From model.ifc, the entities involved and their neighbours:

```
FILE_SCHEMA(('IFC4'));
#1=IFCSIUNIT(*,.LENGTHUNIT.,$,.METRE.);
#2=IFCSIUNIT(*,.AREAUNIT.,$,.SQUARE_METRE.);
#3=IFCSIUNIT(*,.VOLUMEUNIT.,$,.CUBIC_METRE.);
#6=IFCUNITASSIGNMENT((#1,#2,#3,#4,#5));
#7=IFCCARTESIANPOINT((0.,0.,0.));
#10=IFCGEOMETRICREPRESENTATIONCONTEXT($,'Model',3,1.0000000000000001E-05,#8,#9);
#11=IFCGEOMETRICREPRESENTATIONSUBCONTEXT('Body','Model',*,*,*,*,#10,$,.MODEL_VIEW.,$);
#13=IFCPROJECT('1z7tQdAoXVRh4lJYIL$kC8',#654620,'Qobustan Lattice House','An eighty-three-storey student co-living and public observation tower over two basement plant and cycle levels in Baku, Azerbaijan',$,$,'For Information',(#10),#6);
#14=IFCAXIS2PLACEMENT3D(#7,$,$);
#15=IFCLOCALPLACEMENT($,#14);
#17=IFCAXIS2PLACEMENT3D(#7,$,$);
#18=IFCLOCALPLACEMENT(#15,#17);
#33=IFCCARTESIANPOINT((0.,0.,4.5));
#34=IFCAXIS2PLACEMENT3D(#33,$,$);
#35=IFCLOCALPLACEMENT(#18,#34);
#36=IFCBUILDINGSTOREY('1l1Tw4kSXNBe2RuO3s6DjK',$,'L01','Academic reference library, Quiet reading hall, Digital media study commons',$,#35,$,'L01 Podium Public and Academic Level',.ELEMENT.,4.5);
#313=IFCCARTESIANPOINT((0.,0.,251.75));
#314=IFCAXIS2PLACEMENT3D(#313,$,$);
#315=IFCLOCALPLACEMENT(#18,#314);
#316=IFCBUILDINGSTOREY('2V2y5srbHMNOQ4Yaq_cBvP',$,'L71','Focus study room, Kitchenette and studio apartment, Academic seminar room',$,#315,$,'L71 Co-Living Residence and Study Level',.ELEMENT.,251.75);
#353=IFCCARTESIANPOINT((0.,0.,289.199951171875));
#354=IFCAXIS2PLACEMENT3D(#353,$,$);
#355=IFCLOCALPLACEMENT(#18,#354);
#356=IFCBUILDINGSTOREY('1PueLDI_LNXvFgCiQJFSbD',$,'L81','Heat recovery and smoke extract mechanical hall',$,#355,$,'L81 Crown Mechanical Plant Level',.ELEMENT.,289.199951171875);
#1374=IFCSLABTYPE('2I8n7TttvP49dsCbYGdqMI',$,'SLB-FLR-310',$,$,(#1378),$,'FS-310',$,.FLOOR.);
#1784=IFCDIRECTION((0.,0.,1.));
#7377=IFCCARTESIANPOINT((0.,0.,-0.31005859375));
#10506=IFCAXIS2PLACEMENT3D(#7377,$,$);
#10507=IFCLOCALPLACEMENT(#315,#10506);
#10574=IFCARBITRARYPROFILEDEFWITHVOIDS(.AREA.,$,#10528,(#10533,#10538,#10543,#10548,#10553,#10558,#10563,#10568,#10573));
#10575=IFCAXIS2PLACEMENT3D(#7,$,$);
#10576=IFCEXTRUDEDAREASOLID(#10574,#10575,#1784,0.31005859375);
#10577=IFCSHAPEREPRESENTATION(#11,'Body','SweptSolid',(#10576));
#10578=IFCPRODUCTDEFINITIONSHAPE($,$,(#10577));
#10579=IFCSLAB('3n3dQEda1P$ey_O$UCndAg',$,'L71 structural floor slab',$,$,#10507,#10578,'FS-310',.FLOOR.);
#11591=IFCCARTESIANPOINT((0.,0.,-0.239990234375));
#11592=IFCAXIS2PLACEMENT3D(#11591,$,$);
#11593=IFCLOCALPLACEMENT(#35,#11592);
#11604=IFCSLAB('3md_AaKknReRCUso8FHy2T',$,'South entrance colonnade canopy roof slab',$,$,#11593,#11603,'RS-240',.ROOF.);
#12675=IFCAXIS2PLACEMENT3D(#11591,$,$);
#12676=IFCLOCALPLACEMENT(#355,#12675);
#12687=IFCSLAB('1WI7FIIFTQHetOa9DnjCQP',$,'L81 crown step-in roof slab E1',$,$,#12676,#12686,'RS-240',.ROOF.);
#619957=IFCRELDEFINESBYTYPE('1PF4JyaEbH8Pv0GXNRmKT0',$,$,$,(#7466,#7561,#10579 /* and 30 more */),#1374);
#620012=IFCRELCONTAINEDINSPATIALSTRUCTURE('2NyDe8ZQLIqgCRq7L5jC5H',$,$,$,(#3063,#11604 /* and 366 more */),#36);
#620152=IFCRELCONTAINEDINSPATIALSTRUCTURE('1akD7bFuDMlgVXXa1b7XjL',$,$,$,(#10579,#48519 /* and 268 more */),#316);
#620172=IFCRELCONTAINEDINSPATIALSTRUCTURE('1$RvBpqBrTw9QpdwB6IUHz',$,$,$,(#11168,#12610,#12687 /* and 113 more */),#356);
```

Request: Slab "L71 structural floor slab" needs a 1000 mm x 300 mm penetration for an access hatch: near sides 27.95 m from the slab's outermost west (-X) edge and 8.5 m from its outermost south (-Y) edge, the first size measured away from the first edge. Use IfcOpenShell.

```python
import numpy as np
import ifcopenshell
import ifcopenshell.api.feature
import ifcopenshell.api.geometry
import ifcopenshell.api.root
import ifcopenshell.geom
import ifcopenshell.util.placement
import ifcopenshell.util.representation
import ifcopenshell.util.shape
import ifcopenshell.util.unit

model = ifcopenshell.open("model.ifc")
unit_scale = ifcopenshell.util.unit.calculate_unit_scale(model)
settings = ifcopenshell.geom.settings()


def volume(element):
    """Net volume in cubic metres, openings subtracted."""
    shape = ifcopenshell.geom.create_shape(settings, element)
    return ifcopenshell.util.shape.get_volume(shape.geometry)


slab = model.by_guid("3n3dQEda1P$ey_O$UCndAg")
before = volume(slab)

# Extent in the slab's own axes, in metres. The edges named are its -X and -Y sides.
slab_shape = ifcopenshell.geom.create_shape(settings, slab)
vertices = ifcopenshell.util.shape.get_vertices(slab_shape.geometry)
x_min, y_min, bottom = vertices.min(axis=0)
top = vertices[:, 2].max()

opening = ifcopenshell.api.root.create_entity(model, ifc_class="IfcOpeningElement", name="Access hatch opening", predefined_type="OPENING")
context = ifcopenshell.util.representation.get_context(model, "Model", "Body", "MODEL_VIEW")
width, depth = 1, 0.3
outline = [(0.0, 0.0), (width, 0.0), (width, depth), (0.0, depth), (0.0, 0.0)]
# Overshoot both faces by 50 mm so the cut is clean.
shape = ifcopenshell.api.geometry.add_slab_representation(
    model, context=context, depth=top - bottom + 0.1, polyline=outline
)
ifcopenshell.api.geometry.assign_representation(model, product=opening, representation=shape)

matrix = ifcopenshell.util.placement.get_local_placement(slab.ObjectPlacement)
matrix[:, 3] = matrix @ np.append(np.array([x_min + 27.95, y_min + 8.5, bottom - 0.05]) / unit_scale, 1.0)
ifcopenshell.api.geometry.edit_object_placement(model, product=opening, matrix=matrix, is_si=False)
ifcopenshell.api.feature.add_feature(model, feature=opening, element=slab)

after = volume(slab)

print(f"slab volume {before:.3f} -> {after:.3f} m3")

model.write("model_v2.ifc")
```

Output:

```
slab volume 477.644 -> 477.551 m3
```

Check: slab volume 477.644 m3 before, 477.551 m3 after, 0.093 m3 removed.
